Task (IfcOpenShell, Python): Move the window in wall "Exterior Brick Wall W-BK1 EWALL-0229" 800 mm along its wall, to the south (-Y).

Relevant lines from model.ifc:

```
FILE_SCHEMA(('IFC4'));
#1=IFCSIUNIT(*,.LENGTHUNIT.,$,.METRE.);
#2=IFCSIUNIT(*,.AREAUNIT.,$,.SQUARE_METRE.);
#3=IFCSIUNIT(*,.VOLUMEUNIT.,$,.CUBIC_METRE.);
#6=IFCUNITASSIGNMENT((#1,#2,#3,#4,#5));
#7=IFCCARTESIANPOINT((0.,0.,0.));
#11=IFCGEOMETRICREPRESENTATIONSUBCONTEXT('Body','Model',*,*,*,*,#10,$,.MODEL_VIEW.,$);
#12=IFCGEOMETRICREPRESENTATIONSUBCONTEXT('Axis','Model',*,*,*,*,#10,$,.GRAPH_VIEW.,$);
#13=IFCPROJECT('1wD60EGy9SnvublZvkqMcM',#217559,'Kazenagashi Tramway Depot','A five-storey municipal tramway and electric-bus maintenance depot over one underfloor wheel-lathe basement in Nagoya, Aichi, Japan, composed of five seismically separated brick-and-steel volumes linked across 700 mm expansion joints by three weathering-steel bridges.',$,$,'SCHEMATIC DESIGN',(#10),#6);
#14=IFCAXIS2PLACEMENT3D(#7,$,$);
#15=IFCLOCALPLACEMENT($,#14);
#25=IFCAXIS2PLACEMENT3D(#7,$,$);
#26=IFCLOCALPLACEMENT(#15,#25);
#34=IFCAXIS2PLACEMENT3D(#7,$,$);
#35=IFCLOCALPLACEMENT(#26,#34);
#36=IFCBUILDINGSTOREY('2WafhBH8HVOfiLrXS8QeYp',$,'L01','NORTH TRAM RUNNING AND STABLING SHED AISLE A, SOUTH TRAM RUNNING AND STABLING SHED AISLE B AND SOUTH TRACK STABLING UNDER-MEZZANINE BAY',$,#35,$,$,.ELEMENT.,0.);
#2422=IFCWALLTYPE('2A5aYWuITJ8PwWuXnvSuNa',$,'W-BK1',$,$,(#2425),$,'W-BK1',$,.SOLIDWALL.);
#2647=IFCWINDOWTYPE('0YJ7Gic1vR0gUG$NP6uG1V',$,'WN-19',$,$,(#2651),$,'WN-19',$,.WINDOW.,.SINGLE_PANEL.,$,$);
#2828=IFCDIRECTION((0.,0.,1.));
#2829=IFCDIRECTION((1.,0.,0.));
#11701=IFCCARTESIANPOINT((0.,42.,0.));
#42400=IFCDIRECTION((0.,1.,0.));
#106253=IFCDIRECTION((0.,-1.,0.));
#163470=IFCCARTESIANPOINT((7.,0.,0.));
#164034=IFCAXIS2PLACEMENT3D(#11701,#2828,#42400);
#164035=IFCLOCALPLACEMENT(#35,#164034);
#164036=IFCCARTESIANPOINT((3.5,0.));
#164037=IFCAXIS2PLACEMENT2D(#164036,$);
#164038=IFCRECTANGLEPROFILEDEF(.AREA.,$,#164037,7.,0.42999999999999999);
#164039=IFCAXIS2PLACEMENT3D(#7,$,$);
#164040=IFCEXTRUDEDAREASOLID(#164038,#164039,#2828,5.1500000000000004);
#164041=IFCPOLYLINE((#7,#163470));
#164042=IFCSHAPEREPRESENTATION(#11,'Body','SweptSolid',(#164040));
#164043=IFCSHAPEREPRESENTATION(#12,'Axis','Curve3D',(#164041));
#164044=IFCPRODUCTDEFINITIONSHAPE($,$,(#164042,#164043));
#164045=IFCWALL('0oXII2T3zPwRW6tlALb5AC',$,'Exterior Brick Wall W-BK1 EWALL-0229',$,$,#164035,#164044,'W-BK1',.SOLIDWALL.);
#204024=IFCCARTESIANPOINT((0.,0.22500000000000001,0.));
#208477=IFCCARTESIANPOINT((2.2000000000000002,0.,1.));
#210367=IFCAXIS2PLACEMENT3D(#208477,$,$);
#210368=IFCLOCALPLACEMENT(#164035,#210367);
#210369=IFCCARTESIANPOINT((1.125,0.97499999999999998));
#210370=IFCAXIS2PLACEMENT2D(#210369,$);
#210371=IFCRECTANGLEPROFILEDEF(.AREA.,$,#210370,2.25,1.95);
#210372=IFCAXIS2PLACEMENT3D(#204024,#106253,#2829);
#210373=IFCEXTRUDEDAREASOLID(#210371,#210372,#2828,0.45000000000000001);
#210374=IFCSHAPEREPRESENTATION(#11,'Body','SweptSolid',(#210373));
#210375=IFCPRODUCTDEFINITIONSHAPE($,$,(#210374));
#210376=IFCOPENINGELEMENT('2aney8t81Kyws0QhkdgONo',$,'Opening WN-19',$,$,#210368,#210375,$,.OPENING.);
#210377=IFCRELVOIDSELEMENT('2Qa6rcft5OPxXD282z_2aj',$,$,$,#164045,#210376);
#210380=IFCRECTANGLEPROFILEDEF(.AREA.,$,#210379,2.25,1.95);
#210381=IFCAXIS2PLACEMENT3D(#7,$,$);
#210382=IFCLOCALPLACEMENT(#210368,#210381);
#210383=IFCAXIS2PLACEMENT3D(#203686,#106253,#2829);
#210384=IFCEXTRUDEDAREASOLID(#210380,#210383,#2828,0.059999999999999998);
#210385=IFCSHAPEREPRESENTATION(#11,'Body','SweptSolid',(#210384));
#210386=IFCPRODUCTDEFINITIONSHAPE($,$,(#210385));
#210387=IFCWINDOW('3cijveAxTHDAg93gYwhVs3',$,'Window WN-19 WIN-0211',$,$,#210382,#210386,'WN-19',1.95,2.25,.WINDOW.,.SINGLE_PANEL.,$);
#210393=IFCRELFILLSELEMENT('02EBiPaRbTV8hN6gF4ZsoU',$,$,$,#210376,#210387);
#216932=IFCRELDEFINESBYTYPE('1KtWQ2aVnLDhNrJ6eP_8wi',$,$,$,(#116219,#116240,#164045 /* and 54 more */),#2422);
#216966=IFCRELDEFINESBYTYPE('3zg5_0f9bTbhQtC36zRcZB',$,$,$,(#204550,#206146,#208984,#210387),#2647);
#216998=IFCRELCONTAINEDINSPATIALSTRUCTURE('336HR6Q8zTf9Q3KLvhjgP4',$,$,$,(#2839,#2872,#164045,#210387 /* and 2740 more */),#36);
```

```python
import ifcopenshell
import ifcopenshell.api.geometry
import ifcopenshell.util.placement
import ifcopenshell.util.unit

model = ifcopenshell.open("model.ifc")
unit_scale = ifcopenshell.util.unit.calculate_unit_scale(model)

window = model.by_id(210387)
opening = window.FillsVoids[0].RelatingOpeningElement
wall = opening.VoidsElements[0].RelatingBuildingElement

wall_matrix = ifcopenshell.util.placement.get_local_placement(wall.ObjectPlacement)
shift = wall_matrix[:3, 0] * -0.8 / unit_scale
before = ifcopenshell.util.placement.get_local_placement(window.ObjectPlacement)[:3, 3].copy()

# The window is placed relative to its opening, so it follows when the opening moves.
matrix = ifcopenshell.util.placement.get_local_placement(opening.ObjectPlacement)
matrix[:3, 3] += shift
ifcopenshell.api.geometry.edit_object_placement(
    model, product=opening, matrix=matrix, is_si=False, should_transform_children=True
)

after = ifcopenshell.util.placement.get_local_placement(window.ObjectPlacement)[:3, 3]
print("window moved by", (after - before).round(3) + 0.0)

model.write("model_edited.ifc")
```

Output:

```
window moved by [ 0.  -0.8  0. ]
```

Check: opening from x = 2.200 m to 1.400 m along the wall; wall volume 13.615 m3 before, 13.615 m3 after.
